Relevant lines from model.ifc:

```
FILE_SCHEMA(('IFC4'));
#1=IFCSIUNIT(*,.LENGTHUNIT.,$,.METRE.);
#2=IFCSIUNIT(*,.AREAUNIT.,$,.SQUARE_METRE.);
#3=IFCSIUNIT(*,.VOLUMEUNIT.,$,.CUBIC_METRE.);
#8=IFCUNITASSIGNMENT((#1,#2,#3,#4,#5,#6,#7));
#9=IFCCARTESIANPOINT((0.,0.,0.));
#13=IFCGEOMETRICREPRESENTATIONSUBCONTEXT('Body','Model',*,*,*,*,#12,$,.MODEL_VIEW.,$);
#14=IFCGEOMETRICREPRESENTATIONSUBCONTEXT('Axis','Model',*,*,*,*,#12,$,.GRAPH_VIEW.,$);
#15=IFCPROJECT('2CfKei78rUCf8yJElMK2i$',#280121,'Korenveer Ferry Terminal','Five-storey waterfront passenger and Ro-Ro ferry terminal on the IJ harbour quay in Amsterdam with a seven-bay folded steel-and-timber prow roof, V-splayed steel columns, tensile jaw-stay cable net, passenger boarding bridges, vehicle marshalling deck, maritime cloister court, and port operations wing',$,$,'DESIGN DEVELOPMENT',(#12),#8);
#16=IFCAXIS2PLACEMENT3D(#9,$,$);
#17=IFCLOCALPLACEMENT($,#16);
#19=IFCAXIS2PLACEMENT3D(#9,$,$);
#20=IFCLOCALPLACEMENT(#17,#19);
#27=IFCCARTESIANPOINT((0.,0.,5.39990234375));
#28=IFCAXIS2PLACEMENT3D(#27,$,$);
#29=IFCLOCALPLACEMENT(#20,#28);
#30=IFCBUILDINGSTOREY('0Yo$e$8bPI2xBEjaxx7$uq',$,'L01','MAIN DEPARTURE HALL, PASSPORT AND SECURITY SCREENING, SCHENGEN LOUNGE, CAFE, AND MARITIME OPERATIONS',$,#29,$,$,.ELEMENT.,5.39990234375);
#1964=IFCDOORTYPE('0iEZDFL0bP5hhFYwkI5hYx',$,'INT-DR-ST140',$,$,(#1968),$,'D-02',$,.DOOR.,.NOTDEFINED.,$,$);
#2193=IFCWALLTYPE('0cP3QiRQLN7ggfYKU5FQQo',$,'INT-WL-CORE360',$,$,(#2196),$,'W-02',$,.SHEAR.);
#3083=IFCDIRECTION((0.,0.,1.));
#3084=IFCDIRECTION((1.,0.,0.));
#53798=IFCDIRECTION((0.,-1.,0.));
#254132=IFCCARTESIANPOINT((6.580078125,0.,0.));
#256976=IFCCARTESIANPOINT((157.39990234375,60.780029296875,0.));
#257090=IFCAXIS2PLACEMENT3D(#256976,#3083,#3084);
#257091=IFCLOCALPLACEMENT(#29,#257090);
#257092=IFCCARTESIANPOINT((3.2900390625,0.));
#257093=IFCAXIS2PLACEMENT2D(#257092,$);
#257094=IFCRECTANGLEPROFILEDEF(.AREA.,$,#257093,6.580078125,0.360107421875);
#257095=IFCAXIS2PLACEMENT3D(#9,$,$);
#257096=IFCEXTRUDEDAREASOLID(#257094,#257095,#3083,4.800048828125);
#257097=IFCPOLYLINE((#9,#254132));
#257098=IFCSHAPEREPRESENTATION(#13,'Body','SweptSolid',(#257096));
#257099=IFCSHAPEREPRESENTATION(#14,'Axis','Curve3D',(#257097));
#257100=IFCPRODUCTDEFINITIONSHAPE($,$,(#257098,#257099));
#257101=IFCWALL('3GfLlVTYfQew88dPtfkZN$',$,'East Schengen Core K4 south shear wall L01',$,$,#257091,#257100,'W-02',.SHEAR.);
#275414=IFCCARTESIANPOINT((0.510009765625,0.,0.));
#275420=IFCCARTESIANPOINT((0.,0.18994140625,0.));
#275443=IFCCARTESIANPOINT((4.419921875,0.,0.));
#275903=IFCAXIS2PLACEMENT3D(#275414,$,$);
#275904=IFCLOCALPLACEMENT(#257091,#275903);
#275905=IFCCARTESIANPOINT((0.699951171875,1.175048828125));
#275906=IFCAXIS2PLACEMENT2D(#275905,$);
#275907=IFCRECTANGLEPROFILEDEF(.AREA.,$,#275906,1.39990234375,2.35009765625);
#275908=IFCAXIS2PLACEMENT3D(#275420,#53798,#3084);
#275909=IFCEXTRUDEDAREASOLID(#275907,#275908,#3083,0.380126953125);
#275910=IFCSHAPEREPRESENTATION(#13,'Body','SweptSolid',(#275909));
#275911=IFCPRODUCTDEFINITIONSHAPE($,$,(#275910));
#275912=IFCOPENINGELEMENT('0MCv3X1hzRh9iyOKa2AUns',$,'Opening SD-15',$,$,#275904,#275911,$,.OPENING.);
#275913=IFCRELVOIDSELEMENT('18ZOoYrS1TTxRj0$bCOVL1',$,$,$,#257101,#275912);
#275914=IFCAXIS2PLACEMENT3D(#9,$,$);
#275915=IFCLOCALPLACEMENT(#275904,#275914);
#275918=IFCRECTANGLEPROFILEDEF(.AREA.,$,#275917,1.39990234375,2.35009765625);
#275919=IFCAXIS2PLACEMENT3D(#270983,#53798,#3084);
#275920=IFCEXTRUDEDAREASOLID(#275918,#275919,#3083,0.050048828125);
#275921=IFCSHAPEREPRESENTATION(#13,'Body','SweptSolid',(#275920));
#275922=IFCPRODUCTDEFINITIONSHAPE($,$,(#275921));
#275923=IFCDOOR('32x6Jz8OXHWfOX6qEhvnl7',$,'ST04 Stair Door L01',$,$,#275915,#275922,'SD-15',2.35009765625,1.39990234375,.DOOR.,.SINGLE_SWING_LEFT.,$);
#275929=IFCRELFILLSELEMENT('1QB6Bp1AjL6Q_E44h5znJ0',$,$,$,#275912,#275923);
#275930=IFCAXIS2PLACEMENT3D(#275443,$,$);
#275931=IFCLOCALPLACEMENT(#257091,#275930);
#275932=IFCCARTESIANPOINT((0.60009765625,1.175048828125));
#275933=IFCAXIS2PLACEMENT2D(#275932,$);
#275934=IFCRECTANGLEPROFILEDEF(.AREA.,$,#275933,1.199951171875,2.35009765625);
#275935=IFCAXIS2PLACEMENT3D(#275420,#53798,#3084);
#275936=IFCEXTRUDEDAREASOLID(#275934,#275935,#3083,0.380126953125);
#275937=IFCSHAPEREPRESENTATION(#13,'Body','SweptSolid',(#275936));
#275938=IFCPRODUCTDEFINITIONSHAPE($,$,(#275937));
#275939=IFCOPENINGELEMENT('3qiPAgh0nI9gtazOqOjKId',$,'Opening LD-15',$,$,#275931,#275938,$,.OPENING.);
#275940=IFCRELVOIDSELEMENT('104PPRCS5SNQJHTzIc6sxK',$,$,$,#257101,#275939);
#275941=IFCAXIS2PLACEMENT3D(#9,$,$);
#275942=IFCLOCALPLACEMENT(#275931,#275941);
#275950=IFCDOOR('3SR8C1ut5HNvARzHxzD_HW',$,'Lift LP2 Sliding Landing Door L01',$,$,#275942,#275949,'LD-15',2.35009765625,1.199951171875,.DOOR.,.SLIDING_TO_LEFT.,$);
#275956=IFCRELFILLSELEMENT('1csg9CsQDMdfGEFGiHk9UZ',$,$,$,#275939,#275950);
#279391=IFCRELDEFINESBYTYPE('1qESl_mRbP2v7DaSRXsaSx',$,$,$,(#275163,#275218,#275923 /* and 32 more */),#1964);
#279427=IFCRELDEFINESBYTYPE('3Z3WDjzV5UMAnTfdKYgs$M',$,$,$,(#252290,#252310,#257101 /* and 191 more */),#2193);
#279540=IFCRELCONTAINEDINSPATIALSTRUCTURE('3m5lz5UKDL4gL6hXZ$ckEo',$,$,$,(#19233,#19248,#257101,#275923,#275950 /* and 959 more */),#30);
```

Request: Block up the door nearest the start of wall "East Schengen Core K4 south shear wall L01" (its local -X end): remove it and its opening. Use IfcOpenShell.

```python
import ifcopenshell
import ifcopenshell.api.feature
import ifcopenshell.api.root
import ifcopenshell.geom
import ifcopenshell.util.shape

model = ifcopenshell.open("model.ifc")
settings = ifcopenshell.geom.settings()


def volume(element):
    """Net volume in cubic metres, openings subtracted."""
    shape = ifcopenshell.geom.create_shape(settings, element)
    return ifcopenshell.util.shape.get_volume(shape.geometry)


door = model.by_guid("32x6Jz8OXHWfOX6qEhvnl7")
opening = door.FillsVoids[0].RelatingOpeningElement
wall = opening.VoidsElements[0].RelatingBuildingElement
before = volume(wall)

ifcopenshell.api.root.remove_product(model, product=door)
ifcopenshell.api.feature.remove_feature(model, feature=opening)

after = volume(wall)

print(f"wall volume {before:.3f} -> {after:.3f} m3")

model.write("model_rev.ifc")
```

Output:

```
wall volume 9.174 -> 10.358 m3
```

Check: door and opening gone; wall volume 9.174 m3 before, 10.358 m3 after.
